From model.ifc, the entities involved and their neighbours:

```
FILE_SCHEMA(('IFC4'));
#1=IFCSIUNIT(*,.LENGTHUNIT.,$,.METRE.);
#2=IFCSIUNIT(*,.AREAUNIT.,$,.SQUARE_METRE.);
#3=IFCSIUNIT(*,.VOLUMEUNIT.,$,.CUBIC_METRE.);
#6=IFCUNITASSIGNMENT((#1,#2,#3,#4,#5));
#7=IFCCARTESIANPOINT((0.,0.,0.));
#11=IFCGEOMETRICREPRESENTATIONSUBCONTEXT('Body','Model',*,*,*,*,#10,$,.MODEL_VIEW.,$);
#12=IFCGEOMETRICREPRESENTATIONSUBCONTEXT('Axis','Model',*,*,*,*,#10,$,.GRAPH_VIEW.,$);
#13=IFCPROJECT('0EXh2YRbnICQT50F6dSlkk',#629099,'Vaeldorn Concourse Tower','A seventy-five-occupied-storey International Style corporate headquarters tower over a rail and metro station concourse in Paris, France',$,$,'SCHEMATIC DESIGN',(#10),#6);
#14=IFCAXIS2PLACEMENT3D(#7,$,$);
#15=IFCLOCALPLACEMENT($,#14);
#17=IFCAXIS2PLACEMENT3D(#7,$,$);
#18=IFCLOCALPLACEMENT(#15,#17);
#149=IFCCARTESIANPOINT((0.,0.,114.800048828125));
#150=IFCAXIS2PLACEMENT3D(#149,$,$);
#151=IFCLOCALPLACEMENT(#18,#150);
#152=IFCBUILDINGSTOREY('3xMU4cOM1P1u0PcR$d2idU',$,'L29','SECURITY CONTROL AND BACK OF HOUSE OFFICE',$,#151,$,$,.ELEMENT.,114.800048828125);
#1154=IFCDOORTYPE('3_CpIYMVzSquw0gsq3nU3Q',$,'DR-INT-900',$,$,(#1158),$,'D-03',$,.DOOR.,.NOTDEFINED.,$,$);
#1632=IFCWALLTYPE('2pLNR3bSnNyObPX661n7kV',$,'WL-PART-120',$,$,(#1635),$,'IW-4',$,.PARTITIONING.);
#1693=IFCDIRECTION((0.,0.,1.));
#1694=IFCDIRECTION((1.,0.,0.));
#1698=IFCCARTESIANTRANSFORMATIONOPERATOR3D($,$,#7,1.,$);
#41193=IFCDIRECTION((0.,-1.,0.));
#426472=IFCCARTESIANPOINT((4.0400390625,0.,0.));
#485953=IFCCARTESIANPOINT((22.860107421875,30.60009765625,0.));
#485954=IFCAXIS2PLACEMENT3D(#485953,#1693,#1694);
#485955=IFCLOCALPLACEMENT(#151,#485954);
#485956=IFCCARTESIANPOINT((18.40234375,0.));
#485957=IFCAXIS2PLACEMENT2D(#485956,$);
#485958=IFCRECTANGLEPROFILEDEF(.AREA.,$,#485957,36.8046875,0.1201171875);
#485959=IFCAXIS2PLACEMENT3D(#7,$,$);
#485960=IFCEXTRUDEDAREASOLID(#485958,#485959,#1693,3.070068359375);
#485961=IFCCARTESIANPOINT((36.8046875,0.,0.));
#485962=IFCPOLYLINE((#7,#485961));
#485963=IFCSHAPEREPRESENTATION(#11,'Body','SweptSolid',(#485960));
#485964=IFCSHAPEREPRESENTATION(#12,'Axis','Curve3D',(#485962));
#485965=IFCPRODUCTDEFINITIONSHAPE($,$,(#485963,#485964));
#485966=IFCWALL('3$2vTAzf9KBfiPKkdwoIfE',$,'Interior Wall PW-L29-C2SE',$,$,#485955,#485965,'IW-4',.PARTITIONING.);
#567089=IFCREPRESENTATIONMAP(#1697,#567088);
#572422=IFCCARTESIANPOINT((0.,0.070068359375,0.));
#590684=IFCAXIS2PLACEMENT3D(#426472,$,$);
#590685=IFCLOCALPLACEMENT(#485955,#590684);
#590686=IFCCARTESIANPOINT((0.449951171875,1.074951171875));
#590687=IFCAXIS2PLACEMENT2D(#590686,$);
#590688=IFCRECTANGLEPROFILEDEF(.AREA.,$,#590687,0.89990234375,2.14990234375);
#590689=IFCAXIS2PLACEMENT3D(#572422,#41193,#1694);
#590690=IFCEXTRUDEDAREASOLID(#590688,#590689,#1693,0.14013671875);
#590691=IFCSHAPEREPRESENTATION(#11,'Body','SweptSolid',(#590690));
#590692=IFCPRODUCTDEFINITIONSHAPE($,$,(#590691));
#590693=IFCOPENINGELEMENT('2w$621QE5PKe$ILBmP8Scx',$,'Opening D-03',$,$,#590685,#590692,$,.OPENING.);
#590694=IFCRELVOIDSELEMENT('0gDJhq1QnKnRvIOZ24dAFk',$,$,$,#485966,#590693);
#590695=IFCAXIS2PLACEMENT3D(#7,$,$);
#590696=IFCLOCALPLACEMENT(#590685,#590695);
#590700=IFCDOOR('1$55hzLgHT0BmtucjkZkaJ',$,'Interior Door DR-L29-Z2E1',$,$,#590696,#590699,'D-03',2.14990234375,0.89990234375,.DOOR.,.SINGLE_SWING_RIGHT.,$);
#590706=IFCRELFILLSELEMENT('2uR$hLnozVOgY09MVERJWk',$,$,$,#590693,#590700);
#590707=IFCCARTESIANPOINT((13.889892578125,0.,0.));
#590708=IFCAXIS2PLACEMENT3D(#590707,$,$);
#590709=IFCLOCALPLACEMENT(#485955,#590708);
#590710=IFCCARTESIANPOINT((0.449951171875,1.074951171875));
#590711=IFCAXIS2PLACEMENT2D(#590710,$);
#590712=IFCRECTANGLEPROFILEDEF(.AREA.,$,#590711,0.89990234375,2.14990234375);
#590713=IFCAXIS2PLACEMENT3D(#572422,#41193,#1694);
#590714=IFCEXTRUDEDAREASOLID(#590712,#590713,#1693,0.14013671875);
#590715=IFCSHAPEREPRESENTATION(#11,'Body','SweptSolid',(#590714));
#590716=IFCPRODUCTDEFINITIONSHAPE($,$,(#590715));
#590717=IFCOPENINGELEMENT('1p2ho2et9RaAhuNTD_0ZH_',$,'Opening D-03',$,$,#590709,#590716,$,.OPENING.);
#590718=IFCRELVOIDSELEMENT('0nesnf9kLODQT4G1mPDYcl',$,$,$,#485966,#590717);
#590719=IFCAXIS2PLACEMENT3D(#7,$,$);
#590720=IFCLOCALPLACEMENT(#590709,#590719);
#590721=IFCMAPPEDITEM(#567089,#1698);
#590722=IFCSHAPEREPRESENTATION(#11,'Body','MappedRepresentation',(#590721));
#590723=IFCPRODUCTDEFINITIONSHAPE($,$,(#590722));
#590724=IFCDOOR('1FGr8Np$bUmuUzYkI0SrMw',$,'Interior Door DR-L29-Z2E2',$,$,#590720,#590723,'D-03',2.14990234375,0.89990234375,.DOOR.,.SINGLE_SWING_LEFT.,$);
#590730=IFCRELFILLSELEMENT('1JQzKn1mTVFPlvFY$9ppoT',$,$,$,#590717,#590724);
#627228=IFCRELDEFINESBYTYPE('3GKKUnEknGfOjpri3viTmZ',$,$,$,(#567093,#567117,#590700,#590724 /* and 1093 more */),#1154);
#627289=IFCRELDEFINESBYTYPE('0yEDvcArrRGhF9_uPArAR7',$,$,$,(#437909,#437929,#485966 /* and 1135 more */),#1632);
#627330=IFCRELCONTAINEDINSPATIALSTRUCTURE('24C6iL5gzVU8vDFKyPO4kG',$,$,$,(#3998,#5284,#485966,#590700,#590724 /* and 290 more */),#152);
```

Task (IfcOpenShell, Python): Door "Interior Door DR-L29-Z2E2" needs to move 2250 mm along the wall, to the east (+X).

```python
import ifcopenshell
import ifcopenshell.api.geometry
import ifcopenshell.util.placement
import ifcopenshell.util.unit

model = ifcopenshell.open("model.ifc")
unit_scale = ifcopenshell.util.unit.calculate_unit_scale(model)

door = model.by_guid("1FGr8Np$bUmuUzYkI0SrMw")
opening = door.FillsVoids[0].RelatingOpeningElement
wall = opening.VoidsElements[0].RelatingBuildingElement

wall_matrix = ifcopenshell.util.placement.get_local_placement(wall.ObjectPlacement)
shift = wall_matrix[:3, 0] * 2.25 / unit_scale
before = ifcopenshell.util.placement.get_local_placement(door.ObjectPlacement)[:3, 3].copy()

# The door is placed relative to its opening, so it follows when the opening moves.
matrix = ifcopenshell.util.placement.get_local_placement(opening.ObjectPlacement)
matrix[:3, 3] += shift
ifcopenshell.api.geometry.edit_object_placement(
    model, product=opening, matrix=matrix, is_si=False, should_transform_children=True
)

after = ifcopenshell.util.placement.get_local_placement(door.ObjectPlacement)[:3, 3]
print("door moved by", (after - before).round(3) + 0.0)

model.write("model_updated.ifc")
```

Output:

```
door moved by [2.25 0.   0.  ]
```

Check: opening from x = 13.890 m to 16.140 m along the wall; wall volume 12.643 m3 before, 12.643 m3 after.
